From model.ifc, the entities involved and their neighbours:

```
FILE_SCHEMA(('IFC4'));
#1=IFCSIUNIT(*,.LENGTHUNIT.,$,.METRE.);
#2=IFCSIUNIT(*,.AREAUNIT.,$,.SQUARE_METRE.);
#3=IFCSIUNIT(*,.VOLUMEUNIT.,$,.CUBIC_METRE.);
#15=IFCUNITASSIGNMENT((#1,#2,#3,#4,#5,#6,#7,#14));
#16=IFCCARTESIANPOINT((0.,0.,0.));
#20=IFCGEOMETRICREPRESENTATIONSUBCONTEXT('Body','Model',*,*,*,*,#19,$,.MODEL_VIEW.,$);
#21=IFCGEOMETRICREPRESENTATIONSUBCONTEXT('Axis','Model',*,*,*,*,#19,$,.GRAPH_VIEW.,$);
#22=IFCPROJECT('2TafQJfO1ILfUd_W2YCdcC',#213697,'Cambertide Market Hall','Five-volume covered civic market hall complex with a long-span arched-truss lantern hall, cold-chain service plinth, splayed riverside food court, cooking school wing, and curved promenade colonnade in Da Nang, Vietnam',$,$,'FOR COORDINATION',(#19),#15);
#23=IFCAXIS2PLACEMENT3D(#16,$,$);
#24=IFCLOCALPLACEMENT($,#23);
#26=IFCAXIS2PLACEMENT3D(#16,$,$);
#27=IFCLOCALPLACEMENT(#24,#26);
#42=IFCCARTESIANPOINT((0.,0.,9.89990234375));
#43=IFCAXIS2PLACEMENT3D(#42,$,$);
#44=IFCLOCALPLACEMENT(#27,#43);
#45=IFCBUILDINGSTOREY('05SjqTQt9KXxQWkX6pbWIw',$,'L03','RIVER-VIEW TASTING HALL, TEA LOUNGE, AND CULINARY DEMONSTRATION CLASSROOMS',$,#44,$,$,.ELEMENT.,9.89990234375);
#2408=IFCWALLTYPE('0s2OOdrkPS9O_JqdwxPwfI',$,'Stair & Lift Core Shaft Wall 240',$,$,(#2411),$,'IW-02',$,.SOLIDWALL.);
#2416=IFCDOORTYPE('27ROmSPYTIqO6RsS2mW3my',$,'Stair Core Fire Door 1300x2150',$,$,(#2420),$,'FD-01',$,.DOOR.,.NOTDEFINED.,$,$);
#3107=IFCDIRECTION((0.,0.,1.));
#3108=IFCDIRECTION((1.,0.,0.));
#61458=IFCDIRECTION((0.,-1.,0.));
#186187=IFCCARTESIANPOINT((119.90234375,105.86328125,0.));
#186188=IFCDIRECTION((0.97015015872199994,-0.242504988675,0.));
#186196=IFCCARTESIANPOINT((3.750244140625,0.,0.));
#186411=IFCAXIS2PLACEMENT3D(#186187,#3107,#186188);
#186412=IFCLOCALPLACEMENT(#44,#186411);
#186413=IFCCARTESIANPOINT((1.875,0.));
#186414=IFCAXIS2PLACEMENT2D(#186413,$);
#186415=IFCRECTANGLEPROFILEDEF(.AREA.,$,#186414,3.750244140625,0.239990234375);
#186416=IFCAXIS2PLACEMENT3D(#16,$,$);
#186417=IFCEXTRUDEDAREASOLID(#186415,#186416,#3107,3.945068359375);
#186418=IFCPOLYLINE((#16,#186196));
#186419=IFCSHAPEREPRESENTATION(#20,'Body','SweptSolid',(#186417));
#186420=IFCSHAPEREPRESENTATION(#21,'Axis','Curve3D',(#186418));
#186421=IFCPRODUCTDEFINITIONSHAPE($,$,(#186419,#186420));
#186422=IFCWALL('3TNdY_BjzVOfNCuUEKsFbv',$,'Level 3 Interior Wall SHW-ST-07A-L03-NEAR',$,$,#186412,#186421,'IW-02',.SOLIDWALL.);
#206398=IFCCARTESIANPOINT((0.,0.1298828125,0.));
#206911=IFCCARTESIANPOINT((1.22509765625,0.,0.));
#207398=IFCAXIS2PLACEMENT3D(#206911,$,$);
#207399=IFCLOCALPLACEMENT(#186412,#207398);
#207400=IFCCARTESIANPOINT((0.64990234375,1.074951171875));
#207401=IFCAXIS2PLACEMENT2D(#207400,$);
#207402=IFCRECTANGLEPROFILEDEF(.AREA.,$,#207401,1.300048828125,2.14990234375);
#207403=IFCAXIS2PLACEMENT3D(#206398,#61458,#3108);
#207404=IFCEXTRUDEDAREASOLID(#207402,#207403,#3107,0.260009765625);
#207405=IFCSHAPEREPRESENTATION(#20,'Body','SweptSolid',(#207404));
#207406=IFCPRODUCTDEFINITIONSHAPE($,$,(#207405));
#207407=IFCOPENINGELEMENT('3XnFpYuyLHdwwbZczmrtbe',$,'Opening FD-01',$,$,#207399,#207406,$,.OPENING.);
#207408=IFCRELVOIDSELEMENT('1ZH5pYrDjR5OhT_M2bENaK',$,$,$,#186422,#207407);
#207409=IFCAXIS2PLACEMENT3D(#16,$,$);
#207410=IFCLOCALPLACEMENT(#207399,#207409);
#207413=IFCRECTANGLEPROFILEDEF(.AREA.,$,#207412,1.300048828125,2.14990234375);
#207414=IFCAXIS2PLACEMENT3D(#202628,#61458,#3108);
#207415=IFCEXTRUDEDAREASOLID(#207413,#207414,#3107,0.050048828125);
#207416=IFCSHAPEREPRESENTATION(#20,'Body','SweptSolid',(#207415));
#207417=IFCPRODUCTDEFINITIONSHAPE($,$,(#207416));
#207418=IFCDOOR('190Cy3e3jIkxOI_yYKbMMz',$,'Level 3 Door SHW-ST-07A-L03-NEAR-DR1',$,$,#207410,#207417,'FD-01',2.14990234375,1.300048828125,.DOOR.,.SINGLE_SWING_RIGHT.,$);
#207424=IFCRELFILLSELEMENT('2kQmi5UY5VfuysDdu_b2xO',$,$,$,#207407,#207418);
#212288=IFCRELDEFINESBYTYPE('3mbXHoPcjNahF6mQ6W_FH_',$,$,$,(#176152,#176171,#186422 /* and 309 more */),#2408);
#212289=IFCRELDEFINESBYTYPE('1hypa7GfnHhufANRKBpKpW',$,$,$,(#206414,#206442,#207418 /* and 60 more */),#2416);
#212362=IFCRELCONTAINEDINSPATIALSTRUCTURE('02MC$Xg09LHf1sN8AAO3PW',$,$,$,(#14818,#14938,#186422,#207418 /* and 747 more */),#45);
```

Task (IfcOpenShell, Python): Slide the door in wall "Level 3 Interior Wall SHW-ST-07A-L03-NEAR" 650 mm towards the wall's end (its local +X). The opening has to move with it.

```python
import ifcopenshell
import ifcopenshell.api.geometry
import ifcopenshell.util.placement
import ifcopenshell.util.unit

model = ifcopenshell.open("model.ifc")
unit_scale = ifcopenshell.util.unit.calculate_unit_scale(model)

door = model.by_guid("190Cy3e3jIkxOI_yYKbMMz")
opening = door.FillsVoids[0].RelatingOpeningElement
wall = opening.VoidsElements[0].RelatingBuildingElement

wall_matrix = ifcopenshell.util.placement.get_local_placement(wall.ObjectPlacement)
shift = wall_matrix[:3, 0] * 0.65 / unit_scale
before = ifcopenshell.util.placement.get_local_placement(door.ObjectPlacement)[:3, 3].copy()

# The door is placed relative to its opening, so it follows when the opening moves.
matrix = ifcopenshell.util.placement.get_local_placement(opening.ObjectPlacement)
matrix[:3, 3] += shift
ifcopenshell.api.geometry.edit_object_placement(
    model, product=opening, matrix=matrix, is_si=False, should_transform_children=True
)

after = ifcopenshell.util.placement.get_local_placement(door.ObjectPlacement)[:3, 3]
print("door moved by", (after - before).round(3) + 0.0)

model.write("model-out.ifc")
```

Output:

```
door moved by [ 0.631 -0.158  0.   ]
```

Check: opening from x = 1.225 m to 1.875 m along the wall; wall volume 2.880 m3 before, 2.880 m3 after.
